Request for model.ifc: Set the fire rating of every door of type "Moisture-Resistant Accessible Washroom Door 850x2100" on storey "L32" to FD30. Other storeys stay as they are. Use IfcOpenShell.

First a look at what the model holds.

```python
import ifcopenshell
import ifcopenshell.util.element

model = ifcopenshell.open("model.ifc")
print(model.schema)
storey = next(s for s in model.by_type("IfcBuildingStorey") if s.Name == "L32")
doors = [e for e in ifcopenshell.util.element.get_decomposition(storey) if e.is_a("IfcDoor")]
seen = {}
for e in doors:
    element_type = ifcopenshell.util.element.get_type(e)
    key = (element_type.Name if element_type != e and element_type else None, ifcopenshell.util.element.get_pset(e, "Pset_DoorCommon", "FireRating"))
    seen[key] = seen.get(key, 0) + 1
for (name, value), count in sorted(seen.items(), key=str):
    print(count, "x", name, "|", value)
```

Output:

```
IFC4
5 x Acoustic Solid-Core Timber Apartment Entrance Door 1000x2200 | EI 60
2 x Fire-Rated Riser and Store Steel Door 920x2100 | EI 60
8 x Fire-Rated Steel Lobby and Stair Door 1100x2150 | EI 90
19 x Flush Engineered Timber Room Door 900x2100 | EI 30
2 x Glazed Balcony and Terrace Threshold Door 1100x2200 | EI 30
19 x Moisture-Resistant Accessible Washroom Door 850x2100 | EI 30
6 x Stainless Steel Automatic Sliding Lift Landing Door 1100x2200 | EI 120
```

```python
import ifcopenshell
import ifcopenshell.api.pset
import ifcopenshell.util.element

model = ifcopenshell.open("model.ifc")

storey = next(s for s in model.by_type("IfcBuildingStorey") if s.Name == "L32")
doors = [e for e in ifcopenshell.util.element.get_decomposition(storey) if e.is_a("IfcDoor")]

count = 0
for e in doors:
    element_type = ifcopenshell.util.element.get_type(e)
    if element_type in (None, e) or element_type.Name != "Moisture-Resistant Accessible Washroom Door 850x2100":
        continue
    found = ifcopenshell.util.element.get_pset(e, "Pset_DoorCommon", should_inherit=False)
    if found:
        pset = model.by_id(found["id"])
        if len(ifcopenshell.util.element.get_elements_by_pset(pset)) > 1:
            pset = ifcopenshell.api.pset.unshare_pset(model, products=[e], pset=pset)[0]
    else:
        pset = ifcopenshell.api.pset.add_pset(model, product=e, name="Pset_DoorCommon")
    ifcopenshell.api.pset.edit_pset(model, pset=pset, properties={"FireRating": "FD30"})
    count += 1

print(count, "doors updated")

model.write("model_v2.ifc")
```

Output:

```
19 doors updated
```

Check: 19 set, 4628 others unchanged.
